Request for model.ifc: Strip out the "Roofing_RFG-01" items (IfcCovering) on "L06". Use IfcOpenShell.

First a look at what the model holds.

```python
import ifcopenshell
import ifcopenshell.util.element

model = ifcopenshell.open("model.ifc")
print(model.schema)
storey = next(s for s in model.by_type("IfcBuildingStorey") if s.Name == "L06")
coverings = [e for e in ifcopenshell.util.element.get_decomposition(storey) if e.is_a("IfcCovering")]
seen = {}
for e in coverings:
    element_type = ifcopenshell.util.element.get_type(e)
    name = element_type.Name if element_type not in (None, e) else None
    seen[name] = seen.get(name, 0) + 1
for name, count in sorted(seen.items(), key=str):
    print(count, "x", name)
```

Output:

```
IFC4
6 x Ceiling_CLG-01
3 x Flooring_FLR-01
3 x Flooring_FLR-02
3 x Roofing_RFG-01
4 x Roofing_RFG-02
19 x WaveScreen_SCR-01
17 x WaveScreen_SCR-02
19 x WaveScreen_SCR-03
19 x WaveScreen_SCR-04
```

```python
import ifcopenshell
import ifcopenshell.api.root
import ifcopenshell.util.element

model = ifcopenshell.open("model.ifc")

storey = next(s for s in model.by_type("IfcBuildingStorey") if s.Name == "L06")
coverings = [e for e in ifcopenshell.util.element.get_decomposition(storey) if e.is_a("IfcCovering")]
targets = [e for e in coverings if (t := ifcopenshell.util.element.get_type(e)) not in (None, e) and t.Name == "Roofing_RFG-01"]

for e in targets:
    ifcopenshell.api.root.remove_product(model, product=e)
print(len(targets), "removed")

model.write("model_edited.ifc")
```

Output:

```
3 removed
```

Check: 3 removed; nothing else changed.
